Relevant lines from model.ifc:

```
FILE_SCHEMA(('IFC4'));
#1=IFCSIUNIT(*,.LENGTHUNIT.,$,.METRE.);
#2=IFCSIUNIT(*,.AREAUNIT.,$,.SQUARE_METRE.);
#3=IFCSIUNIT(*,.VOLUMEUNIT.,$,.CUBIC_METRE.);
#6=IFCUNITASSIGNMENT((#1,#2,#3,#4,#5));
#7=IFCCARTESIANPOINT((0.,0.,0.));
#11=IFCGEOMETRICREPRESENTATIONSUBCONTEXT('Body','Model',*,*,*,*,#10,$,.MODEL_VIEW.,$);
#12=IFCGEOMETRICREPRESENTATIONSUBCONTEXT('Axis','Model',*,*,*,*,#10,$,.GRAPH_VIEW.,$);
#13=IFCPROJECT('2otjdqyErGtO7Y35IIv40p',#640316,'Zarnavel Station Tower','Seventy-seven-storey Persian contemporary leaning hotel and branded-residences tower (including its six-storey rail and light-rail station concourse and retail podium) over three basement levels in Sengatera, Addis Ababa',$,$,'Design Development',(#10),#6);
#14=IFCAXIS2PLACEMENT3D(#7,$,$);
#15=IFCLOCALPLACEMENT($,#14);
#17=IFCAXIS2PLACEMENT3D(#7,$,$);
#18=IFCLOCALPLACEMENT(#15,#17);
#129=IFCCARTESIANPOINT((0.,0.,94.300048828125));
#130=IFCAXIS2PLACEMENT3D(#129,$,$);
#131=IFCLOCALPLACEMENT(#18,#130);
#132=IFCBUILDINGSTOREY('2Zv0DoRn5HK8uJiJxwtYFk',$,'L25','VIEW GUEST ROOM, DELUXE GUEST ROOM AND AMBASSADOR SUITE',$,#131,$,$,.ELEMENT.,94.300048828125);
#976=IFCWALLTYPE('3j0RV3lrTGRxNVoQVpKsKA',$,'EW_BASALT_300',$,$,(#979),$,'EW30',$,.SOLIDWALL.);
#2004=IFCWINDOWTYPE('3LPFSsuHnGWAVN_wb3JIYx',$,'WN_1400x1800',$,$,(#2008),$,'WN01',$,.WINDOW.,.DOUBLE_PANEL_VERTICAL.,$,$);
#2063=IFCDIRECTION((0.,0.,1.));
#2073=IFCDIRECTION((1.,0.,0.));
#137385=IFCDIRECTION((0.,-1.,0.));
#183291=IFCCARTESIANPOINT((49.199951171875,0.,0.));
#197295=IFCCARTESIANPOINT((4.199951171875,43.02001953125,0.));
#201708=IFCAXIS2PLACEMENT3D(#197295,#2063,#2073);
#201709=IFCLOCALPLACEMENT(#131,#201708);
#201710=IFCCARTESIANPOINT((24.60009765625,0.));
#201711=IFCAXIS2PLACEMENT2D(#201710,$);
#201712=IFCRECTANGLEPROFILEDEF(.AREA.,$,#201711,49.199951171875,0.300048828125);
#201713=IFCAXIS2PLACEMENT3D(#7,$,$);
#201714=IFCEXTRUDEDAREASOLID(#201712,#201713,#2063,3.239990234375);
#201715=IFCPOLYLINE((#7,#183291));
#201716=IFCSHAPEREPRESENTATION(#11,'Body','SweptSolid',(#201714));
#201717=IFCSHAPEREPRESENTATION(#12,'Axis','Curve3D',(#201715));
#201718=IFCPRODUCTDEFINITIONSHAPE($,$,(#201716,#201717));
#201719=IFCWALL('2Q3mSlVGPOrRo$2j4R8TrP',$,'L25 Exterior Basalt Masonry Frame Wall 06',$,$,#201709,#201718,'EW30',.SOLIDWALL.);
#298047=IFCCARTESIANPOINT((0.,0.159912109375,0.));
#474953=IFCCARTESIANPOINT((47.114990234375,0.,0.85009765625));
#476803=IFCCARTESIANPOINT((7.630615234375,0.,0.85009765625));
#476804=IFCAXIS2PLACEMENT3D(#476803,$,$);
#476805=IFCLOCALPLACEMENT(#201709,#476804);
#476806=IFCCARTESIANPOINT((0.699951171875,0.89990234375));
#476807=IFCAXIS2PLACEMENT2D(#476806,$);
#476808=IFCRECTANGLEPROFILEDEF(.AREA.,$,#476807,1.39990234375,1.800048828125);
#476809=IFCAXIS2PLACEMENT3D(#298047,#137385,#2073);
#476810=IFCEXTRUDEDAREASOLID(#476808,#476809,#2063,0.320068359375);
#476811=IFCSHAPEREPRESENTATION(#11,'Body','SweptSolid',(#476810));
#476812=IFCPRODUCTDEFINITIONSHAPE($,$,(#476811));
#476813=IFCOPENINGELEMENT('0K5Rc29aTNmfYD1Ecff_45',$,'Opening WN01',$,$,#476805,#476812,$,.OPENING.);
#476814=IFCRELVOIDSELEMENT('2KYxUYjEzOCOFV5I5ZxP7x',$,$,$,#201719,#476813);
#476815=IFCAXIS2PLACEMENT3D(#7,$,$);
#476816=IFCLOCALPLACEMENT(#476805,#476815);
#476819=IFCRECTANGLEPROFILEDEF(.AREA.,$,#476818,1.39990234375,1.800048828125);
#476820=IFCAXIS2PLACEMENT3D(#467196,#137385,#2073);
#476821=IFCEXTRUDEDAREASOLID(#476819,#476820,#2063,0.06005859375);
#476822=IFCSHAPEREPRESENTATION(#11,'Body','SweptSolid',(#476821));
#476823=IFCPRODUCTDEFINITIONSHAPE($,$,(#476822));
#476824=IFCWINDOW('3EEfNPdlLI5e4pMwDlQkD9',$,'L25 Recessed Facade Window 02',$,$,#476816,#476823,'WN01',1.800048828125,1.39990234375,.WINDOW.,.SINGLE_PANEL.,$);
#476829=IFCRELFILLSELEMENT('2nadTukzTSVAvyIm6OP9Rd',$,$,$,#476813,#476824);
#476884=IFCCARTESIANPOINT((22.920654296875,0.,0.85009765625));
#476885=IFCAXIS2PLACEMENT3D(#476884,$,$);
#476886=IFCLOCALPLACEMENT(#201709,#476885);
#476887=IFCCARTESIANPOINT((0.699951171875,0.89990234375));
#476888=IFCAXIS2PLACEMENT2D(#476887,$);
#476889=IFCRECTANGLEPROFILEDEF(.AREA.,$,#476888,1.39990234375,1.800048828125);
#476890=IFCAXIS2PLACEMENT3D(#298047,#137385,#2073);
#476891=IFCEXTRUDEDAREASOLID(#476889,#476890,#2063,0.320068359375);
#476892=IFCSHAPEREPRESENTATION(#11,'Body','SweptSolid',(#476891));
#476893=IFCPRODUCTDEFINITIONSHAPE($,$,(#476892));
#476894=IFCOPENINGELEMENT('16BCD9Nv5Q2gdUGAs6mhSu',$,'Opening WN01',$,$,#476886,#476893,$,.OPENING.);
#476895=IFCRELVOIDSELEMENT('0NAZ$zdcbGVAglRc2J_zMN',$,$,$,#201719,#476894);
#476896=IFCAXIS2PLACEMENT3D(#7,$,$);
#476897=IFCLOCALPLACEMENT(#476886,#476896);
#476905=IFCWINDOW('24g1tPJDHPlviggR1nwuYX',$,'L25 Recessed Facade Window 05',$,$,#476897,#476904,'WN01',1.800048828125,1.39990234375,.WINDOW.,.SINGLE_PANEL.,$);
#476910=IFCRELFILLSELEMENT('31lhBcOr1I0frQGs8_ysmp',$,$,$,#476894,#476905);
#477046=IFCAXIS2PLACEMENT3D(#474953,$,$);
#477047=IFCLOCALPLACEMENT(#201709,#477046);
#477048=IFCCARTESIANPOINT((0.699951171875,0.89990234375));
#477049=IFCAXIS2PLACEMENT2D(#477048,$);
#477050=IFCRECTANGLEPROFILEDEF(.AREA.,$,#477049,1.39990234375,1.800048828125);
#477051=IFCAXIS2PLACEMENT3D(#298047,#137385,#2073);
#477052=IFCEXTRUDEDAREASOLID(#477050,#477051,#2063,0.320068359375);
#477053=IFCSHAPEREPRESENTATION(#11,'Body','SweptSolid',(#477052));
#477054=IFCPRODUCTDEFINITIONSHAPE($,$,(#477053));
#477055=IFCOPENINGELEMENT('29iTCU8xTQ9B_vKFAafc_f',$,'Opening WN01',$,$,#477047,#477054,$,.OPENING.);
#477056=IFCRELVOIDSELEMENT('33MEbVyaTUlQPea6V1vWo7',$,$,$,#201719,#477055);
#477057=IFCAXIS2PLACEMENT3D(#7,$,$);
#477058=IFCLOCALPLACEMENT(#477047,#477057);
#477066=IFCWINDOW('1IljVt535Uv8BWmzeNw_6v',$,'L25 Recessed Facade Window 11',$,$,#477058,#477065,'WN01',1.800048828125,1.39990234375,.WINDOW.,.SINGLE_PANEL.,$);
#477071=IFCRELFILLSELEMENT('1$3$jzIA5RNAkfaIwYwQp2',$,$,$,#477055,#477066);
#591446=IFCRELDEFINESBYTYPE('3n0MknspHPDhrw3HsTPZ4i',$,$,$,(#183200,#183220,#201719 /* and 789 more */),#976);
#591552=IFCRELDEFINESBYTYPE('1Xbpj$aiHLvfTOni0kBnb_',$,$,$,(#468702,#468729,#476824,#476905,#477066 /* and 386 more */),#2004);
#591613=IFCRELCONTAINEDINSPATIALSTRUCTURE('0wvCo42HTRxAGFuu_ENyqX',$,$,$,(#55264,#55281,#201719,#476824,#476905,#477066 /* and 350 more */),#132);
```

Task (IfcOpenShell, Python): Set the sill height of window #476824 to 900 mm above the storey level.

```python
import numpy as np
import ifcopenshell
import ifcopenshell.api.geometry
import ifcopenshell.geom
import ifcopenshell.util.element
import ifcopenshell.util.placement
import ifcopenshell.util.shape
import ifcopenshell.util.unit

model = ifcopenshell.open("model.ifc")
unit_scale = ifcopenshell.util.unit.calculate_unit_scale(model)

window = model.by_guid("3EEfNPdlLI5e4pMwDlQkD9")
opening = window.FillsVoids[0].RelatingOpeningElement
storey = ifcopenshell.util.element.get_container(window, ifc_class="IfcBuildingStorey")
level = ifcopenshell.util.placement.get_local_placement(storey.ObjectPlacement)[2, 3]

# The opening's origin need not be at the sill, so measure its lowest point.
shape = ifcopenshell.geom.create_shape(ifcopenshell.geom.settings(), opening)
bottom = ifcopenshell.util.shape.get_shape_bottom_elevation(shape, shape.geometry) / unit_scale
dz = level + 0.9 - bottom

shift = np.array([0.0, 0.0, dz])
# The window is placed relative to its opening, so it follows when the opening moves.
matrix = ifcopenshell.util.placement.get_local_placement(opening.ObjectPlacement)
matrix[:3, 3] += shift
ifcopenshell.api.geometry.edit_object_placement(
    model, product=opening, matrix=matrix, is_si=False, should_transform_children=True
)

print(f"moved by {dz * unit_scale:+.3f} m")

model.write("model_updated.ifc")
```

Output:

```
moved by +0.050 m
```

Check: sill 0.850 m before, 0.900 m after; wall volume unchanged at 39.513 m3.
